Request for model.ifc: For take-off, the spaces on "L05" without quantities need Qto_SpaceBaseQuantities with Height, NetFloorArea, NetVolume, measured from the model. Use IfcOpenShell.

First a look at what the model holds.

```python
import ifcopenshell
import ifcopenshell.util.element
import ifcopenshell.util.unit

model = ifcopenshell.open("model.ifc")
print(model.schema)
for unit_type in ("LENGTHUNIT", "AREAUNIT", "VOLUMEUNIT"):
    print(unit_type, ifcopenshell.util.unit.calculate_unit_scale(model, unit_type))
storey = next(s for s in model.by_type("IfcBuildingStorey") if s.Name == "L05")
spaces = [e for e in ifcopenshell.util.element.get_decomposition(storey) if e.is_a("IfcSpace")]
for e in sorted(spaces, key=lambda e: e.id()):
    print(e.id(), e.is_a(), e.Name, list(ifcopenshell.util.element.get_psets(e, qtos_only=True)), sep=" | ")
```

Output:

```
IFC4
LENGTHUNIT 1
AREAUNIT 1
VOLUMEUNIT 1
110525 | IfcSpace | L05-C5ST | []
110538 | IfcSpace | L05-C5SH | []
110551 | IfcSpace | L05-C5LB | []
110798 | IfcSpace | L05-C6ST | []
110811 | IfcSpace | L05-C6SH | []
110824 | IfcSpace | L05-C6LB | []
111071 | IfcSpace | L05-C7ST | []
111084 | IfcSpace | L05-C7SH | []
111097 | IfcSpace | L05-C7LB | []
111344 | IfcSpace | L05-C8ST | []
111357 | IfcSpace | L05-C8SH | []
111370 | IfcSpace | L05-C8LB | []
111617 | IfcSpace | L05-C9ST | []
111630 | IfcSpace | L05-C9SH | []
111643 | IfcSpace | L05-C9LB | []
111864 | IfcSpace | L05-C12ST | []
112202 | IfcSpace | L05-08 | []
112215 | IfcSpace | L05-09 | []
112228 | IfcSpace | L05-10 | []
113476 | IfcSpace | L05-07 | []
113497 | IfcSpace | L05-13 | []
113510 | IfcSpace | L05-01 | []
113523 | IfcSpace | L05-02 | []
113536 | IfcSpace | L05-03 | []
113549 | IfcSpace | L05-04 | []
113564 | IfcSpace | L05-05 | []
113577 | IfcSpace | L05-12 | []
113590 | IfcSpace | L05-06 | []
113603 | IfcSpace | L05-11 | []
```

```python
import ifcopenshell
import ifcopenshell.api.pset
import ifcopenshell.geom
import ifcopenshell.util.element
import ifcopenshell.util.shape
import ifcopenshell.util.unit

model = ifcopenshell.open("model.ifc")
unit_scale = ifcopenshell.util.unit.calculate_unit_scale(model)
area_scale = ifcopenshell.util.unit.calculate_unit_scale(model, "AREAUNIT")
volume_scale = ifcopenshell.util.unit.calculate_unit_scale(model, "VOLUMEUNIT")
settings = ifcopenshell.geom.settings()

storey = next(s for s in model.by_type("IfcBuildingStorey") if s.Name == "L05")
spaces = [e for e in ifcopenshell.util.element.get_decomposition(storey) if e.is_a("IfcSpace")]

for e in sorted(spaces, key=lambda e: e.id()):
    if ifcopenshell.util.element.get_psets(e, qtos_only=True, should_inherit=False):
        continue
    # Geometry comes back in metres, in the element's own axes.
    shape = ifcopenshell.geom.create_shape(settings, e)
    values = {
        "Height": ifcopenshell.util.shape.get_z(shape.geometry) / unit_scale,
        "NetFloorArea": ifcopenshell.util.shape.get_footprint_area(shape.geometry) / area_scale,
        "NetVolume": ifcopenshell.util.shape.get_volume(shape.geometry) / volume_scale,
    }
    qto = ifcopenshell.api.pset.add_qto(model, product=e, name="Qto_SpaceBaseQuantities")
    ifcopenshell.api.pset.edit_qto(model, qto=qto, properties=values)
    print(e.id(), {k: round(v, 3) for k, v in values.items()})

model.write("model_v2.ifc")
```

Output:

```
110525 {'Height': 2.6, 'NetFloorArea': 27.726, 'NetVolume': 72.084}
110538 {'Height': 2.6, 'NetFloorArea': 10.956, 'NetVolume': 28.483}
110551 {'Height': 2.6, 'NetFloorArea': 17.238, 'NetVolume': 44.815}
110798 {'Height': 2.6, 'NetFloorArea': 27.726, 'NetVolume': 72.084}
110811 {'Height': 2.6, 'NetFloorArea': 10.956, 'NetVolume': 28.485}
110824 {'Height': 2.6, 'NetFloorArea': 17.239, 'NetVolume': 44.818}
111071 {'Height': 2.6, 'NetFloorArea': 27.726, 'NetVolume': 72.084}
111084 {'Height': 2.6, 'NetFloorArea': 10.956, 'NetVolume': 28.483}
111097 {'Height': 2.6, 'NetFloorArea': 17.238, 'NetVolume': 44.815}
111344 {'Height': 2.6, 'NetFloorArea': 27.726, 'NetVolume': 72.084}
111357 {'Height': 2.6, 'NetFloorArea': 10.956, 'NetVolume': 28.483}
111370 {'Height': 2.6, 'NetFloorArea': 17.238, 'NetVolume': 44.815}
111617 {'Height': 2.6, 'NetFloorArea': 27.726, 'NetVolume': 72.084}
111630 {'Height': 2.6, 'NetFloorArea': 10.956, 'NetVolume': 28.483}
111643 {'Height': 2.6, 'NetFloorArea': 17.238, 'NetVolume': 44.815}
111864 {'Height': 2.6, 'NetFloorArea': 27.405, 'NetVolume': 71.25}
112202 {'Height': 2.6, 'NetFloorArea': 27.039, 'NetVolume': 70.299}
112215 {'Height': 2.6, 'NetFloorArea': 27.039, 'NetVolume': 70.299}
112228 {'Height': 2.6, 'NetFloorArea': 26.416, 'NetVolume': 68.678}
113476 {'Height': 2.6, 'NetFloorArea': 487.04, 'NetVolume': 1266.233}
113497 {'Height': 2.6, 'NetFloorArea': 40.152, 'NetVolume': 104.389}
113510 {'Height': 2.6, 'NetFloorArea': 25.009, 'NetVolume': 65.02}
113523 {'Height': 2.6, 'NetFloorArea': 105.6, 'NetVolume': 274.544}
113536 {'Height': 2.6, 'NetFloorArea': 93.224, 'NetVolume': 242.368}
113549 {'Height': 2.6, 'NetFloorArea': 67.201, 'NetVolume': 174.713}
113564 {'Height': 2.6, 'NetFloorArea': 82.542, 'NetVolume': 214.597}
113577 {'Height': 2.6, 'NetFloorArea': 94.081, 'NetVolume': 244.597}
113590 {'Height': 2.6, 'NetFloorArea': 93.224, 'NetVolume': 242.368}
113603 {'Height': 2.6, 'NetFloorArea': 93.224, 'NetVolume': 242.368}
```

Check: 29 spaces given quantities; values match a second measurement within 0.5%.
